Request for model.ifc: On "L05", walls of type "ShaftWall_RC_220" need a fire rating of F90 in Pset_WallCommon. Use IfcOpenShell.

First a look at what the model holds.

```python
import ifcopenshell
import ifcopenshell.util.element

model = ifcopenshell.open("model.ifc")
print(model.schema)
storey = next(s for s in model.by_type("IfcBuildingStorey") if s.Name == "L05")
walls = [e for e in ifcopenshell.util.element.get_decomposition(storey) if e.is_a("IfcWall")]
seen = {}
for e in walls:
    element_type = ifcopenshell.util.element.get_type(e)
    key = (element_type.Name if element_type != e and element_type else None, ifcopenshell.util.element.get_pset(e, "Pset_WallCommon", "FireRating"))
    seen[key] = seen.get(key, 0) + 1
for (name, value), count in sorted(seen.items(), key=str):
    print(count, "x", name, "|", value)
```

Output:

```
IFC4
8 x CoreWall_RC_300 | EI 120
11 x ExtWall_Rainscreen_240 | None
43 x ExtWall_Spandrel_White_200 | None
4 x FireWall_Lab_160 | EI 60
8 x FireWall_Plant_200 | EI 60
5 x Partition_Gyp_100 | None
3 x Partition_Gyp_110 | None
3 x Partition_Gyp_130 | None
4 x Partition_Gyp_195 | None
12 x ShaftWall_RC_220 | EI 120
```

```python
import ifcopenshell
import ifcopenshell.api.pset
import ifcopenshell.util.element

model = ifcopenshell.open("model.ifc")

storey = next(s for s in model.by_type("IfcBuildingStorey") if s.Name == "L05")
walls = [e for e in ifcopenshell.util.element.get_decomposition(storey) if e.is_a("IfcWall")]

count = 0
for e in walls:
    element_type = ifcopenshell.util.element.get_type(e)
    if element_type in (None, e) or element_type.Name != "ShaftWall_RC_220":
        continue
    # add_pset returns the element's existing set when there is one.
    pset = ifcopenshell.api.pset.add_pset(model, product=e, name="Pset_WallCommon")
    ifcopenshell.api.pset.edit_pset(model, pset=pset, properties={"FireRating": "F90"})
    count += 1

print(count, "walls updated")

model.write("model_edited.ifc")
```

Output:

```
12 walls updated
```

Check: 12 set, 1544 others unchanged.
